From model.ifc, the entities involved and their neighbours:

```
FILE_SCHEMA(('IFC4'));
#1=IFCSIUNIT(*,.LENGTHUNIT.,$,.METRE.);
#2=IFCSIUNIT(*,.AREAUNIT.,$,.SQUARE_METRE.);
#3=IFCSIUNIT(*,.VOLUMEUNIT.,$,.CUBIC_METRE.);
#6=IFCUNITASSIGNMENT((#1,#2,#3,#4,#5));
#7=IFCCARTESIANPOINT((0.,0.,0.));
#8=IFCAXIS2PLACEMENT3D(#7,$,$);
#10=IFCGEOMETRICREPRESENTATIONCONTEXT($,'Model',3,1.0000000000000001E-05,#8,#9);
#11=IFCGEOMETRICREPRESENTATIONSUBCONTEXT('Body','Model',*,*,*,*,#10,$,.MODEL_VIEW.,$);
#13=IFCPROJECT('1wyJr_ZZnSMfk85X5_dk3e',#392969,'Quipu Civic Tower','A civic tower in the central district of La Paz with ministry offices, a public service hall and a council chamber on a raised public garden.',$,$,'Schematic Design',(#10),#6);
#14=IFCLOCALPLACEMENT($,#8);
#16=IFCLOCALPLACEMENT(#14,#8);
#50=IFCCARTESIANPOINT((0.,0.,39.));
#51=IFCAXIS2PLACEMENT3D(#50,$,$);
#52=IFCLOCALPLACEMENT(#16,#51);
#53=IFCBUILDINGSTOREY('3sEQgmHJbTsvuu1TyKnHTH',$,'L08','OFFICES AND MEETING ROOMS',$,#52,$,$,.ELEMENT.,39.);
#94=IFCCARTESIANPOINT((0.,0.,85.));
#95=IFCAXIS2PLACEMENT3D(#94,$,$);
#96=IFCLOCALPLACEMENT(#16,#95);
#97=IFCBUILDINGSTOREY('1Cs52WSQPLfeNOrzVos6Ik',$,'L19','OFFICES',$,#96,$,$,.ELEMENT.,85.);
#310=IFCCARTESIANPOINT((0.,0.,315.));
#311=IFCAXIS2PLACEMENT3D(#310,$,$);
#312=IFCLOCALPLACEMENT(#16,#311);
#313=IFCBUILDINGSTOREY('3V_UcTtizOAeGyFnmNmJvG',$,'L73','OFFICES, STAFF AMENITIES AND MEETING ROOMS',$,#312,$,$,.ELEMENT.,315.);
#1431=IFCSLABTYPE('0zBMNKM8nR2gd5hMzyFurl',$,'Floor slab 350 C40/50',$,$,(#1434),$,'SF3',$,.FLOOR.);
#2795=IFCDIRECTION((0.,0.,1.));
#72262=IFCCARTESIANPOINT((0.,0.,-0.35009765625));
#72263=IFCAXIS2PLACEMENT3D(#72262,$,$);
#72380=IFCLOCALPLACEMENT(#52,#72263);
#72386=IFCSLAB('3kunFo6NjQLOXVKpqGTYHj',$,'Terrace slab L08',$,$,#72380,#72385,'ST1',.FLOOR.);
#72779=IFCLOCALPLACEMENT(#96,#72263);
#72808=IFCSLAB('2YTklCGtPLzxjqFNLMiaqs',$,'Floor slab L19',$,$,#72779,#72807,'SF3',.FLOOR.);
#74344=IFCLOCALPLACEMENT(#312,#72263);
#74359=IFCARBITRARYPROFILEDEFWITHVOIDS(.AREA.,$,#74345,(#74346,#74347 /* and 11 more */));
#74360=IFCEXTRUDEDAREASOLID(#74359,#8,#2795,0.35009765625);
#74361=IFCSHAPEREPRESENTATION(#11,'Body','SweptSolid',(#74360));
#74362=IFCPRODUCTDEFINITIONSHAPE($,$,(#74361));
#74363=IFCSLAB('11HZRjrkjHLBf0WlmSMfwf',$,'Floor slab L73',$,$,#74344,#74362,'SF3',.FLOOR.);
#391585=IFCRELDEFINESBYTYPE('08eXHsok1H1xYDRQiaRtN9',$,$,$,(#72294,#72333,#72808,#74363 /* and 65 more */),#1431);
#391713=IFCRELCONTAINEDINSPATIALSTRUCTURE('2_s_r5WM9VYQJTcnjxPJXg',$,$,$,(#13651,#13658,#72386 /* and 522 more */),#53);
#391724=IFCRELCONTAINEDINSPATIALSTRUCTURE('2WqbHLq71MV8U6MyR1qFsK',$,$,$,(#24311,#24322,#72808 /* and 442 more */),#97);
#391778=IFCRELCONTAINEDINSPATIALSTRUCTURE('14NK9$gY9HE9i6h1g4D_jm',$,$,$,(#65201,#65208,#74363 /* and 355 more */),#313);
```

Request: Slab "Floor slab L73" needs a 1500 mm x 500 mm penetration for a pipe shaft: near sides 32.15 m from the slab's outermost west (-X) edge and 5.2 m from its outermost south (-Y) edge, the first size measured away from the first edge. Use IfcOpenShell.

```python
import numpy as np
import ifcopenshell
import ifcopenshell.api.feature
import ifcopenshell.api.geometry
import ifcopenshell.api.root
import ifcopenshell.geom
import ifcopenshell.util.placement
import ifcopenshell.util.representation
import ifcopenshell.util.shape
import ifcopenshell.util.unit

model = ifcopenshell.open("model.ifc")
unit_scale = ifcopenshell.util.unit.calculate_unit_scale(model)
settings = ifcopenshell.geom.settings()


def volume(element):
    """Net volume in cubic metres, openings subtracted."""
    shape = ifcopenshell.geom.create_shape(settings, element)
    return ifcopenshell.util.shape.get_volume(shape.geometry)


slab = model.by_guid("11HZRjrkjHLBf0WlmSMfwf")
before = volume(slab)

# Extent in the slab's own axes, in metres. The edges named are its -X and -Y sides.
slab_shape = ifcopenshell.geom.create_shape(settings, slab)
vertices = ifcopenshell.util.shape.get_vertices(slab_shape.geometry)
x_min, y_min, bottom = vertices.min(axis=0)
top = vertices[:, 2].max()

opening = ifcopenshell.api.root.create_entity(model, ifc_class="IfcOpeningElement", name="Pipe shaft opening", predefined_type="OPENING")
context = ifcopenshell.util.representation.get_context(model, "Model", "Body", "MODEL_VIEW")
width, depth = 1.5, 0.5
outline = [(0.0, 0.0), (width, 0.0), (width, depth), (0.0, depth), (0.0, 0.0)]
# Overshoot both faces by 50 mm so the cut is clean.
shape = ifcopenshell.api.geometry.add_slab_representation(
    model, context=context, depth=top - bottom + 0.1, polyline=outline
)
ifcopenshell.api.geometry.assign_representation(model, product=opening, representation=shape)

matrix = ifcopenshell.util.placement.get_local_placement(slab.ObjectPlacement)
matrix[:, 3] = matrix @ np.append(np.array([x_min + 32.15, y_min + 5.2, bottom - 0.05]) / unit_scale, 1.0)
ifcopenshell.api.geometry.edit_object_placement(model, product=opening, matrix=matrix, is_si=False)
ifcopenshell.api.feature.add_feature(model, feature=opening, element=slab)

after = volume(slab)

print(f"slab volume {before:.3f} -> {after:.3f} m3")

model.write("model-out.ifc")
```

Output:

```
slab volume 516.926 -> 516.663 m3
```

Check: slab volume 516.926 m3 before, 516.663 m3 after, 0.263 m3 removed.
